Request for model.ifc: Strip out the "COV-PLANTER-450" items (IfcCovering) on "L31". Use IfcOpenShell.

First a look at what the model holds.

```python
import ifcopenshell
import ifcopenshell.util.element

model = ifcopenshell.open("model.ifc")
print(model.schema)
storey = next(s for s in model.by_type("IfcBuildingStorey") if s.Name == "L31")
coverings = [e for e in ifcopenshell.util.element.get_decomposition(storey) if e.is_a("IfcCovering")]
seen = {}
for e in coverings:
    element_type = ifcopenshell.util.element.get_type(e)
    name = element_type.Name if element_type not in (None, e) else None
    seen[name] = seen.get(name, 0) + 1
for name, count in sorted(seen.items(), key=str):
    print(count, "x", name)
```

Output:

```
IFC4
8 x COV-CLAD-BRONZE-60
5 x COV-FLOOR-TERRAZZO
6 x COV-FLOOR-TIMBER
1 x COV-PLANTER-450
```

```python
import ifcopenshell
import ifcopenshell.api.root
import ifcopenshell.util.element

model = ifcopenshell.open("model.ifc")

storey = next(s for s in model.by_type("IfcBuildingStorey") if s.Name == "L31")
coverings = [e for e in ifcopenshell.util.element.get_decomposition(storey) if e.is_a("IfcCovering")]
targets = [e for e in coverings if (t := ifcopenshell.util.element.get_type(e)) not in (None, e) and t.Name == "COV-PLANTER-450"]

for e in targets:
    ifcopenshell.api.root.remove_product(model, product=e)
print(len(targets), "removed")

model.write("model_edited.ifc")
```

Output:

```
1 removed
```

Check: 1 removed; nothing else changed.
